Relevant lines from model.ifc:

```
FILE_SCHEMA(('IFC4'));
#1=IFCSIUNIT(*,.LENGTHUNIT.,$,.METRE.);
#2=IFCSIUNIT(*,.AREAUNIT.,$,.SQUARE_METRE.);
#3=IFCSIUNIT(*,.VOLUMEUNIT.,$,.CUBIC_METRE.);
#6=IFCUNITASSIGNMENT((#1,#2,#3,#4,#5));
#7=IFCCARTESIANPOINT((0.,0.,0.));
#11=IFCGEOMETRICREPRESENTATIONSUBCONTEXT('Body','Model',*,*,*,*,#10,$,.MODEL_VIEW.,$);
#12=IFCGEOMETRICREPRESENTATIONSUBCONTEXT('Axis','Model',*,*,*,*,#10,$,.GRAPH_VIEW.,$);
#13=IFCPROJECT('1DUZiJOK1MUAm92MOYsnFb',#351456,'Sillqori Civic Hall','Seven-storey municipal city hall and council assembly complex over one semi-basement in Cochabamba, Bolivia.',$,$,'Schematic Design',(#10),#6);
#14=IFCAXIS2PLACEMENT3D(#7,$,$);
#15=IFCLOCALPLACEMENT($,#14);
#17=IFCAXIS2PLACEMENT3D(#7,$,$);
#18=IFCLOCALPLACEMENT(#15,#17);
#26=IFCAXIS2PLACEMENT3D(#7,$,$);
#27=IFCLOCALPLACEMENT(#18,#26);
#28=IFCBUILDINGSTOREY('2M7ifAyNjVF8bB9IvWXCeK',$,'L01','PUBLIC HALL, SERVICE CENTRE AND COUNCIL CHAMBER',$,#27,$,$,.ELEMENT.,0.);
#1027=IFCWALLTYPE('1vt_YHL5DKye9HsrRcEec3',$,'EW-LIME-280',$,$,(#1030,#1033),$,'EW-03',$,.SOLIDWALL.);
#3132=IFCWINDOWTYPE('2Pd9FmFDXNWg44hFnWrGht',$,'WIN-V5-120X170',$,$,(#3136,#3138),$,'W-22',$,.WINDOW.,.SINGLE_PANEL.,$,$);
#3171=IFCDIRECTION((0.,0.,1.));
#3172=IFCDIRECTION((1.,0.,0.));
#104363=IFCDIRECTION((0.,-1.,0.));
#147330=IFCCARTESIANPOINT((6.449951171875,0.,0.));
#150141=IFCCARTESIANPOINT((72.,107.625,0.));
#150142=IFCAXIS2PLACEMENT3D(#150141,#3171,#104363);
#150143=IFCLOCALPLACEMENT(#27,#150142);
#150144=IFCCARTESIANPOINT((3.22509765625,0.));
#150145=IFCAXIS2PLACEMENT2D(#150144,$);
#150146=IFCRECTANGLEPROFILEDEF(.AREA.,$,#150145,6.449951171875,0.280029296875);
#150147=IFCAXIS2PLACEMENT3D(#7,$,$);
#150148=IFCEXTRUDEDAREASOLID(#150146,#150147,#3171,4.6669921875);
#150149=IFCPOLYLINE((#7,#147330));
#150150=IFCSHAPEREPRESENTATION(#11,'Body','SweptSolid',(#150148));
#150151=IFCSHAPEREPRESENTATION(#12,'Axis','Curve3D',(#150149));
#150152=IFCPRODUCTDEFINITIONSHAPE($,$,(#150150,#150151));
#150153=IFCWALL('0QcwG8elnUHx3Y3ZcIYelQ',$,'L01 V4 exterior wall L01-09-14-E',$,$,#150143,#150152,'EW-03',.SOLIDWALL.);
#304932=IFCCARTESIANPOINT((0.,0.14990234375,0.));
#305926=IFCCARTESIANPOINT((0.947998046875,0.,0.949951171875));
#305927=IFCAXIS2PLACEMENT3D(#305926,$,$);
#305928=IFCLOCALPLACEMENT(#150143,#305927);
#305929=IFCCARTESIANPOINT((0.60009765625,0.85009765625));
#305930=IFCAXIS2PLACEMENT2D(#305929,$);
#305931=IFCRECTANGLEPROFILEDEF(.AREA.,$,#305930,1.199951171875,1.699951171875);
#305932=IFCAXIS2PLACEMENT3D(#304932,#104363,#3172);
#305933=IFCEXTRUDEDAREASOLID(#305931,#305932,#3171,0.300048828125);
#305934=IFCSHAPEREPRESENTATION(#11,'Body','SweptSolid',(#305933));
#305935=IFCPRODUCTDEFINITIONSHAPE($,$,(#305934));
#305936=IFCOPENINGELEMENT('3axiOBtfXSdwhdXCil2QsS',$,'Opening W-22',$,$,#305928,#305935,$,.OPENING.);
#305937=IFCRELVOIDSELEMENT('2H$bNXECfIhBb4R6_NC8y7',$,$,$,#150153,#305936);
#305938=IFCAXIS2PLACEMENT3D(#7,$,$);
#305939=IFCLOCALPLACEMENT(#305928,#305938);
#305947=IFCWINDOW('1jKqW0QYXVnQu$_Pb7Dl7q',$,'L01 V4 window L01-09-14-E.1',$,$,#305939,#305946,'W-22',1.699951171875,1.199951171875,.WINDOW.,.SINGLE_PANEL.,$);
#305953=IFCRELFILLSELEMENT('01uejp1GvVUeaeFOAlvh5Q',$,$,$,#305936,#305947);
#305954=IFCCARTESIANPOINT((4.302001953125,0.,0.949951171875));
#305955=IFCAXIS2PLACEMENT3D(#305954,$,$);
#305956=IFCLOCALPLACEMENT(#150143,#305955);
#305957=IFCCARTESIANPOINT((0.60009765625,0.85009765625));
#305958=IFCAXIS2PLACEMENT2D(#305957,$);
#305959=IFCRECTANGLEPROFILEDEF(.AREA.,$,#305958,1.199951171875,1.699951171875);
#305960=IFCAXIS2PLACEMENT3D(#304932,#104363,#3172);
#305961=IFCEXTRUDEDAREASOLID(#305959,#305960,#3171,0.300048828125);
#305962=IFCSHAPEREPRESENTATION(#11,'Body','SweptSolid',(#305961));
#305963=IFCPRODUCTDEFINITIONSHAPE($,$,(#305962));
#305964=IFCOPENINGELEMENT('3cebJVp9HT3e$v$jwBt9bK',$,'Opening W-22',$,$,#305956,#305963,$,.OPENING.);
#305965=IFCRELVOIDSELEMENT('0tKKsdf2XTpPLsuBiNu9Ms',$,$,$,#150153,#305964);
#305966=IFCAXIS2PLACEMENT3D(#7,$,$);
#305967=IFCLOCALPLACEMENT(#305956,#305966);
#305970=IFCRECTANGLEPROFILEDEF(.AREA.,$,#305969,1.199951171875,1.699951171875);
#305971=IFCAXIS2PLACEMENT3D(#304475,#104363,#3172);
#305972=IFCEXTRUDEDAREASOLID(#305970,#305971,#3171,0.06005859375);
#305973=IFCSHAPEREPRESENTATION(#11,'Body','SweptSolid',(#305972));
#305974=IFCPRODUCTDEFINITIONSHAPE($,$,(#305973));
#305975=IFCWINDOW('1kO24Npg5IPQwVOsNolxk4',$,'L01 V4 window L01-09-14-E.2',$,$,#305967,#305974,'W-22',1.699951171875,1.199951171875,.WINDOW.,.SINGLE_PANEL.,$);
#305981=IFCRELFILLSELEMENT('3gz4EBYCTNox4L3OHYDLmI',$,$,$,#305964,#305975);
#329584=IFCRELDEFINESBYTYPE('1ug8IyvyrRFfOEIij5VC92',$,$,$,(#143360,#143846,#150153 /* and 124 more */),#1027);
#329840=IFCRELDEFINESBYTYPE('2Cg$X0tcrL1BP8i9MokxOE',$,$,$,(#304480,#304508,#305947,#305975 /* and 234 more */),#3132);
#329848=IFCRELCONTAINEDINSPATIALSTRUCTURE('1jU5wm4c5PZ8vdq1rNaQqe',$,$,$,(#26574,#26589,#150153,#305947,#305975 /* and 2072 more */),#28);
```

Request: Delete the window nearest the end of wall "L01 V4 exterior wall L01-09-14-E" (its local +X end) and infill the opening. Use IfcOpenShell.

```python
import ifcopenshell
import ifcopenshell.api.feature
import ifcopenshell.api.root
import ifcopenshell.geom
import ifcopenshell.util.shape

model = ifcopenshell.open("model.ifc")
settings = ifcopenshell.geom.settings()


def volume(element):
    """Net volume in cubic metres, openings subtracted."""
    shape = ifcopenshell.geom.create_shape(settings, element)
    return ifcopenshell.util.shape.get_volume(shape.geometry)


window = model.by_guid("1kO24Npg5IPQwVOsNolxk4")
opening = window.FillsVoids[0].RelatingOpeningElement
wall = opening.VoidsElements[0].RelatingBuildingElement
before = volume(wall)

ifcopenshell.api.root.remove_product(model, product=window)
ifcopenshell.api.feature.remove_feature(model, feature=opening)

after = volume(wall)

print(f"wall volume {before:.3f} -> {after:.3f} m3")

model.write("model_edited.ifc")
```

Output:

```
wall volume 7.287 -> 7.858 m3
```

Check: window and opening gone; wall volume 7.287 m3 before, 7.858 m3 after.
